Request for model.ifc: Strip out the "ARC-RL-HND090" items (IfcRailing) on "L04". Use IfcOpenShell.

First a look at what the model holds.

```python
import ifcopenshell
import ifcopenshell.util.element

model = ifcopenshell.open("model.ifc")
print(model.schema)
storey = next(s for s in model.by_type("IfcBuildingStorey") if s.Name == "L04")
railings = [e for e in ifcopenshell.util.element.get_decomposition(storey) if e.is_a("IfcRailing")]
seen = {}
for e in railings:
    element_type = ifcopenshell.util.element.get_type(e)
    name = element_type.Name if element_type not in (None, e) else None
    seen[name] = seen.get(name, 0) + 1
for name, count in sorted(seen.items(), key=str):
    print(count, "x", name)
```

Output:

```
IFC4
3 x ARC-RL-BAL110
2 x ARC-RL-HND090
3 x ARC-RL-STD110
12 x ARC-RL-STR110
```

```python
import ifcopenshell
import ifcopenshell.api.root
import ifcopenshell.util.element

model = ifcopenshell.open("model.ifc")

storey = next(s for s in model.by_type("IfcBuildingStorey") if s.Name == "L04")
railings = [e for e in ifcopenshell.util.element.get_decomposition(storey) if e.is_a("IfcRailing")]
targets = [e for e in railings if (t := ifcopenshell.util.element.get_type(e)) not in (None, e) and t.Name == "ARC-RL-HND090"]

for e in targets:
    ifcopenshell.api.root.remove_product(model, product=e)
print(len(targets), "removed")

model.write("model_updated.ifc")
```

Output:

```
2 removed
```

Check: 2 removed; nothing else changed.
